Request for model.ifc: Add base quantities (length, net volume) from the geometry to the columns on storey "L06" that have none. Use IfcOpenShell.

First a look at what the model holds.

```python
import ifcopenshell
import ifcopenshell.util.element
import ifcopenshell.util.unit

model = ifcopenshell.open("model.ifc")
print(model.schema)
for unit_type in ("LENGTHUNIT", "AREAUNIT", "VOLUMEUNIT"):
    print(unit_type, ifcopenshell.util.unit.calculate_unit_scale(model, unit_type))
storey = next(s for s in model.by_type("IfcBuildingStorey") if s.Name == "L06")
columns = [e for e in ifcopenshell.util.element.get_decomposition(storey) if e.is_a("IfcColumn")]
for e in sorted(columns, key=lambda e: e.id()):
    print(e.id(), e.is_a(), e.Name, list(ifcopenshell.util.element.get_psets(e, qtos_only=True)), sep=" | ")
```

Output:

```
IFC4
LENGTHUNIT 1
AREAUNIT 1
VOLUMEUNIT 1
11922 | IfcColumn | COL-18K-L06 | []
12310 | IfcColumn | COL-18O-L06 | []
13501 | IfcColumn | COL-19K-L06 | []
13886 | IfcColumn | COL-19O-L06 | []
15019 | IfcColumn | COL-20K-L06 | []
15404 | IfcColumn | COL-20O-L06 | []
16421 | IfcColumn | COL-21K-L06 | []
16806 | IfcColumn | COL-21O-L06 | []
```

```python
import ifcopenshell
import ifcopenshell.api.pset
import ifcopenshell.geom
import ifcopenshell.util.element
import ifcopenshell.util.shape
import ifcopenshell.util.unit

model = ifcopenshell.open("model.ifc")
unit_scale = ifcopenshell.util.unit.calculate_unit_scale(model)
volume_scale = ifcopenshell.util.unit.calculate_unit_scale(model, "VOLUMEUNIT")
settings = ifcopenshell.geom.settings()

storey = next(s for s in model.by_type("IfcBuildingStorey") if s.Name == "L06")
columns = [e for e in ifcopenshell.util.element.get_decomposition(storey) if e.is_a("IfcColumn")]

for e in sorted(columns, key=lambda e: e.id()):
    if ifcopenshell.util.element.get_psets(e, qtos_only=True, should_inherit=False):
        continue
    # Geometry comes back in metres, in the element's own axes.
    shape = ifcopenshell.geom.create_shape(settings, e)
    values = {
        "Length": ifcopenshell.util.shape.get_z(shape.geometry) / unit_scale,
        "NetVolume": ifcopenshell.util.shape.get_volume(shape.geometry) / volume_scale,
    }
    qto = ifcopenshell.api.pset.add_qto(model, product=e, name="Qto_ColumnBaseQuantities")
    ifcopenshell.api.pset.edit_qto(model, qto=qto, properties=values)
    print(e.id(), {k: round(v, 3) for k, v in values.items()})

model.write("model_updated.ifc")
```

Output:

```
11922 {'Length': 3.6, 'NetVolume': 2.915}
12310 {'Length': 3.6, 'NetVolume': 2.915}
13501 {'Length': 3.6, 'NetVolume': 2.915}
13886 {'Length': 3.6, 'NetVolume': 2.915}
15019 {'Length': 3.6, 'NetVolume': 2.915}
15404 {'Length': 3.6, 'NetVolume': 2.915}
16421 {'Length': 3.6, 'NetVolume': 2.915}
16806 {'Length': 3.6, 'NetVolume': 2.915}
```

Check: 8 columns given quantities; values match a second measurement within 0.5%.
